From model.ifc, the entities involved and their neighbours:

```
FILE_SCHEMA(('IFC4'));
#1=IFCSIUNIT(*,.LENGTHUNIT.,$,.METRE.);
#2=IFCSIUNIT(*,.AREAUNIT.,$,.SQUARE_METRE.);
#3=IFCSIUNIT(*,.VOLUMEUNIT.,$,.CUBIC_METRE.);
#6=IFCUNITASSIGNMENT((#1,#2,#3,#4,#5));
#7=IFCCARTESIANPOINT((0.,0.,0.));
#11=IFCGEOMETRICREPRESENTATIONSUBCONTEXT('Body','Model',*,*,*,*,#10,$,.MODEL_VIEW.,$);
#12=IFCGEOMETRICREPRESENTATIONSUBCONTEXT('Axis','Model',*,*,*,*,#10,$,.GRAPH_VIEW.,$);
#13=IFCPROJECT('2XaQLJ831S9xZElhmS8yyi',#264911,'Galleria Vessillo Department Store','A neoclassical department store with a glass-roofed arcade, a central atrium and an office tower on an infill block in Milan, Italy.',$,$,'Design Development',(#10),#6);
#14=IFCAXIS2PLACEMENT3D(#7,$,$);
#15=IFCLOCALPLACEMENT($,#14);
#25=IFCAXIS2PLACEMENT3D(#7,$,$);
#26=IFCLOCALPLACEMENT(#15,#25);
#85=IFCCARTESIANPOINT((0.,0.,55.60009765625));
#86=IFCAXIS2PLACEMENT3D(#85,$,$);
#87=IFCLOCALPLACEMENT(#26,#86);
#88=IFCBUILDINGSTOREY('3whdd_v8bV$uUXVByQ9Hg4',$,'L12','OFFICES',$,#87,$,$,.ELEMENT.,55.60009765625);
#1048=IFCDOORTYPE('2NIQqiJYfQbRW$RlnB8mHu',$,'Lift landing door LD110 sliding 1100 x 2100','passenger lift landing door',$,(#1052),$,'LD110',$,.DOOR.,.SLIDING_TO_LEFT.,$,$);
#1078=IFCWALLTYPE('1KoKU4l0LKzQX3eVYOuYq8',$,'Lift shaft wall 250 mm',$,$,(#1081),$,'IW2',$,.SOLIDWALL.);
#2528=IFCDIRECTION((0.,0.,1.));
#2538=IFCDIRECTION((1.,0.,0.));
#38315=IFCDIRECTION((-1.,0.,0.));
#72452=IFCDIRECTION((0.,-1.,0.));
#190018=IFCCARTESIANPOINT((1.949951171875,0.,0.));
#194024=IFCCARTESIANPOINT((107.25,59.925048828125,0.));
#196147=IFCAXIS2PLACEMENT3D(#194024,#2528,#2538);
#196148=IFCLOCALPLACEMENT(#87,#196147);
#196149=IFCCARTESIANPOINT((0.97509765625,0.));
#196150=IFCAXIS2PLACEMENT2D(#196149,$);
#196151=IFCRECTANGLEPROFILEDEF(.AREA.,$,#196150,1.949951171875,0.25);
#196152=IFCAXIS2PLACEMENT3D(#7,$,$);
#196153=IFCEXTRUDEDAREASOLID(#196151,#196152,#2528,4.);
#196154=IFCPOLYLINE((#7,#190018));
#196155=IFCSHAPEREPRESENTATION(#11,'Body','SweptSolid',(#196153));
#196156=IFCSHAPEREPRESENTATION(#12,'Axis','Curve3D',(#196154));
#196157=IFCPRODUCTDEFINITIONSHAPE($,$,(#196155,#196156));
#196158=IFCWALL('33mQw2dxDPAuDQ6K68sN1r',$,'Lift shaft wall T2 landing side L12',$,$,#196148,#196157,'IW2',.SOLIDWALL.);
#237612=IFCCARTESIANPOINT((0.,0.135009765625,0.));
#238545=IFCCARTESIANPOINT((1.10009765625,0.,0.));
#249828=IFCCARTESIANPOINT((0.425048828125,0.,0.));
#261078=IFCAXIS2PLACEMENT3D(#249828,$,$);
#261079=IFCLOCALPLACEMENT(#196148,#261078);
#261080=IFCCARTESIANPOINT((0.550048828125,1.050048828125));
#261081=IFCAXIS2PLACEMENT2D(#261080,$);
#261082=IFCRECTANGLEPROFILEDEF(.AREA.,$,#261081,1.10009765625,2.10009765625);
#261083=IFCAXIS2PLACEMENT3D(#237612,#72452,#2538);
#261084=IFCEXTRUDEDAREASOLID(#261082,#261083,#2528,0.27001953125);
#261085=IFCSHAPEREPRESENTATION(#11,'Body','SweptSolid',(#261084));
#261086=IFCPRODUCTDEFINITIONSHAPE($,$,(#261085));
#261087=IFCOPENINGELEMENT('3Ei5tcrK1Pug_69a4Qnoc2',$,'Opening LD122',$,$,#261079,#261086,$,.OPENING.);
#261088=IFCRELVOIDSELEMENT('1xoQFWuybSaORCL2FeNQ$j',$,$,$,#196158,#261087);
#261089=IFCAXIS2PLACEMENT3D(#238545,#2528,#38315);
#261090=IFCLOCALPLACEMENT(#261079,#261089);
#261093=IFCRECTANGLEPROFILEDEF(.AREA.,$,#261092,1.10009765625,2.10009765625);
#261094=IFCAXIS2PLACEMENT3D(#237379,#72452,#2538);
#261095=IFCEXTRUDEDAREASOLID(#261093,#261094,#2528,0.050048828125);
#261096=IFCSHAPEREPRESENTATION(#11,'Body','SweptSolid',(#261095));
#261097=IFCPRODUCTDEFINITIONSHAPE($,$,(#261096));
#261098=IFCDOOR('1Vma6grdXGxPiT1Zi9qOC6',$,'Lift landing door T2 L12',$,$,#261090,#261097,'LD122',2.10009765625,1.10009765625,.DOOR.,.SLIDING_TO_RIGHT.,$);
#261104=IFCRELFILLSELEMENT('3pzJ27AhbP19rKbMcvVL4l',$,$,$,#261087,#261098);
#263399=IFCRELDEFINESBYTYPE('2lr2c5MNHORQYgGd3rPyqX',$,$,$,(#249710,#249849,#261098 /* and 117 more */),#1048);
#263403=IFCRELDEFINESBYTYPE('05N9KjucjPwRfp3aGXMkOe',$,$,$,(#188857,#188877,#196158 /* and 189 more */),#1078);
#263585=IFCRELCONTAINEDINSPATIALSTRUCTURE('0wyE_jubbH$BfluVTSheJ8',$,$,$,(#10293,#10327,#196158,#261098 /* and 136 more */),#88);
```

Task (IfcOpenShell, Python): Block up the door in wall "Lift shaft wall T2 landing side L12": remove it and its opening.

```python
import ifcopenshell
import ifcopenshell.api.feature
import ifcopenshell.api.root
import ifcopenshell.geom
import ifcopenshell.util.shape

model = ifcopenshell.open("model.ifc")
settings = ifcopenshell.geom.settings()


def volume(element):
    """Net volume in cubic metres, openings subtracted."""
    shape = ifcopenshell.geom.create_shape(settings, element)
    return ifcopenshell.util.shape.get_volume(shape.geometry)


door = model.by_guid("1Vma6grdXGxPiT1Zi9qOC6")
opening = door.FillsVoids[0].RelatingOpeningElement
wall = opening.VoidsElements[0].RelatingBuildingElement
before = volume(wall)

ifcopenshell.api.root.remove_product(model, product=door)
ifcopenshell.api.feature.remove_feature(model, feature=opening)

after = volume(wall)

print(f"wall volume {before:.3f} -> {after:.3f} m3")

model.write("model-out.ifc")
```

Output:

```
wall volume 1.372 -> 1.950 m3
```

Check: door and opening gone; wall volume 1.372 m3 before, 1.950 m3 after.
